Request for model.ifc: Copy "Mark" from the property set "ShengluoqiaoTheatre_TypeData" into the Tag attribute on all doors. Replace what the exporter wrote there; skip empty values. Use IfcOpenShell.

First a look at what the model holds.

```python
import ifcopenshell
import ifcopenshell.util.element

model = ifcopenshell.open("model.ifc")
print(model.schema)
doors = model.by_type("IfcDoor")
print(len(doors), "doors")
for e in doors[:8]:
    source = ifcopenshell.util.element.get_pset(e, "ShengluoqiaoTheatre_TypeData", "Mark")
    target = e.Tag
    print(e.id(), repr(source), repr(target), sep=" | ")
```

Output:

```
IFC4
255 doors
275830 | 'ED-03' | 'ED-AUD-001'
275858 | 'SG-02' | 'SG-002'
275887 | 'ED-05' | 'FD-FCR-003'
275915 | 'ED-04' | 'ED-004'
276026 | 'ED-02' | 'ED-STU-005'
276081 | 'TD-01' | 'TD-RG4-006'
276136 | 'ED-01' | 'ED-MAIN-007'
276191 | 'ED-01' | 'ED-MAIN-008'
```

```python
import ifcopenshell
import ifcopenshell.util.element

model = ifcopenshell.open("model.ifc")

count = 0
for e in model.by_type("IfcDoor"):
    value = ifcopenshell.util.element.get_pset(e, "ShengluoqiaoTheatre_TypeData", "Mark")
    current = e.Tag
    if not value or not value.strip() or current == value:
        continue
    e.Tag = value
    count += 1

print(count, "doors updated")

model.write("model-out.ifc")
```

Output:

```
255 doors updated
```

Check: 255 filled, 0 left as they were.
